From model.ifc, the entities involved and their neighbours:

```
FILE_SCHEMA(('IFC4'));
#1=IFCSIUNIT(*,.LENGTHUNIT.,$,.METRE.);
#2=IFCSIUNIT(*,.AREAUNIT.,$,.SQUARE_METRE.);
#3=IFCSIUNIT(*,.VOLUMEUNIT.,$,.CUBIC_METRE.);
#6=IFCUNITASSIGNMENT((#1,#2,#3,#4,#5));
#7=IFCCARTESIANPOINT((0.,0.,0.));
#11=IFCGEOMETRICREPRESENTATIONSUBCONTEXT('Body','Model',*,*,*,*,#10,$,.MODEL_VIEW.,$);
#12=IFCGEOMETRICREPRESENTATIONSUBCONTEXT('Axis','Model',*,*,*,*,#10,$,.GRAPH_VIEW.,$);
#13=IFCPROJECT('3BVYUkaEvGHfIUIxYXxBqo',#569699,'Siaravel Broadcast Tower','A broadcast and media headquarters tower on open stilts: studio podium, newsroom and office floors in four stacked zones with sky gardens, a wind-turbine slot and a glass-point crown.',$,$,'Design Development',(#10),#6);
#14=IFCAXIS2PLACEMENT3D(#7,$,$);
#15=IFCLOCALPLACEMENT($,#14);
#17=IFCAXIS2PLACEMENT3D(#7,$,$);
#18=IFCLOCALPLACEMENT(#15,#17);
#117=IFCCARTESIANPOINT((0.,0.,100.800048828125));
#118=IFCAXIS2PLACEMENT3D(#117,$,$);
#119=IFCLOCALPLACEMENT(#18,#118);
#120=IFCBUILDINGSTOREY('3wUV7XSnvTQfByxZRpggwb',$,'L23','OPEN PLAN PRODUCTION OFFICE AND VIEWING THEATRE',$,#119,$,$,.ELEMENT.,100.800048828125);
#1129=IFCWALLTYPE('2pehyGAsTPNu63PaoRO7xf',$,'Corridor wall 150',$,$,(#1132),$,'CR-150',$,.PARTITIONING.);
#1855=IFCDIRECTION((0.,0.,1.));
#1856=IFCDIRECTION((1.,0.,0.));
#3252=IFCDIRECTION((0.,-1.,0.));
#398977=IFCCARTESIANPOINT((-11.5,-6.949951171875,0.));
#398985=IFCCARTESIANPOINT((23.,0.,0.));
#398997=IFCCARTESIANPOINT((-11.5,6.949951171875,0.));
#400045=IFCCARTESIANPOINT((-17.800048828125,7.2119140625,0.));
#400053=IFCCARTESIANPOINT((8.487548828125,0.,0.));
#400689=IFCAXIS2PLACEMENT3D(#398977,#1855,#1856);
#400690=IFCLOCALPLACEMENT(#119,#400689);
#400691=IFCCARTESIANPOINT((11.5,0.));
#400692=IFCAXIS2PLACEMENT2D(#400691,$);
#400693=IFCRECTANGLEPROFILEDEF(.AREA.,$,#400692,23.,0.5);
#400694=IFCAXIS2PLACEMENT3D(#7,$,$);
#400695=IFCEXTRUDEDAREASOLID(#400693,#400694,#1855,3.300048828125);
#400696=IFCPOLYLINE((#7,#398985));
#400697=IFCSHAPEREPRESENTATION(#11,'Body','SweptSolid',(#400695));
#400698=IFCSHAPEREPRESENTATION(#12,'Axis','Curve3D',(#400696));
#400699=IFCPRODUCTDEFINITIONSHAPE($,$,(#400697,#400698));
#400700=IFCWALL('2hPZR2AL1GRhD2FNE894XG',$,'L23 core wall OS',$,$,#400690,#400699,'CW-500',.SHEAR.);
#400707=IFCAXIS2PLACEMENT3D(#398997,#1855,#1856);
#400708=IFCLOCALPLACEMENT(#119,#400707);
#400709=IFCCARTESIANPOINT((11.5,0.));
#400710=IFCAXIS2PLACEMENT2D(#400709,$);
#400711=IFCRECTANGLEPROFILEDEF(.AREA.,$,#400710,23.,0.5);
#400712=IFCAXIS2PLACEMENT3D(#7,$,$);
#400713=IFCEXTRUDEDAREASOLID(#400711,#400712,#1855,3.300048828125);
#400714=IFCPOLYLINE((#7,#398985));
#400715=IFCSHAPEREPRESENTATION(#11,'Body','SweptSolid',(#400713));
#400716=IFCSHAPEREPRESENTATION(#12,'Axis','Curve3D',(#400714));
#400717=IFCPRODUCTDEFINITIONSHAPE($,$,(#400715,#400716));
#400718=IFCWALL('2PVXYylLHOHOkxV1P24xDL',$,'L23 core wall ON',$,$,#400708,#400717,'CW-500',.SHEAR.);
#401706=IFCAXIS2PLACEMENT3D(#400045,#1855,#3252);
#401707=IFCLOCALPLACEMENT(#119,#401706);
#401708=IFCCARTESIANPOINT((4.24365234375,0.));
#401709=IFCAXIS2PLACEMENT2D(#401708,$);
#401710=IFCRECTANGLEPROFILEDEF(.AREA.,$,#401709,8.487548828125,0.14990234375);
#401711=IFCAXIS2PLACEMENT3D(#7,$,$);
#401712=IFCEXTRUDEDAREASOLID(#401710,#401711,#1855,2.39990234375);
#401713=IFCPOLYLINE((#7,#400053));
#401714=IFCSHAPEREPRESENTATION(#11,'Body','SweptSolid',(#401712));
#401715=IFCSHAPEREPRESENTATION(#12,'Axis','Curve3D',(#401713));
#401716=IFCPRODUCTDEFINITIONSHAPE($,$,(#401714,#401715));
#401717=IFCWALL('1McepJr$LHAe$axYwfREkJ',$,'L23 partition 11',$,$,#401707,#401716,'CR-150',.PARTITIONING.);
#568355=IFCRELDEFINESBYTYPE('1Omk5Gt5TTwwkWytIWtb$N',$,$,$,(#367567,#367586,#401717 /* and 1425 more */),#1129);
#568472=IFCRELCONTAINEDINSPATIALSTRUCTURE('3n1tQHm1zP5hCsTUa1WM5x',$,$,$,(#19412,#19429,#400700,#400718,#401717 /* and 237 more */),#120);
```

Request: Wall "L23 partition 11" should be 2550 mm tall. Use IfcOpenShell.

```python
import ifcopenshell
import ifcopenshell.geom
import ifcopenshell.util.representation
import ifcopenshell.util.shape
import ifcopenshell.util.unit

model = ifcopenshell.open("model.ifc")
unit_scale = ifcopenshell.util.unit.calculate_unit_scale(model)
settings = ifcopenshell.geom.settings()


def volume(element):
    """Net volume in cubic metres, openings subtracted."""
    shape = ifcopenshell.geom.create_shape(settings, element)
    return ifcopenshell.util.shape.get_volume(shape.geometry)


wall = model.by_guid("1McepJr$LHAe$axYwfREkJ")
before = volume(wall)

body = ifcopenshell.util.representation.get_representation(wall, "Model", "Body")
solid = body.Items[0]
old_height = solid.Depth
solid.Depth = 2.55 / unit_scale
after = volume(wall)

print(f"height {old_height:g} -> {solid.Depth:g}, volume {before:.3f} -> {after:.3f} m3")

model.write("model_edited.ifc")
```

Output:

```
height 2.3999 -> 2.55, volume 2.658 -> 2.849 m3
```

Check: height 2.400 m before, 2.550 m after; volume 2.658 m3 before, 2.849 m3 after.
